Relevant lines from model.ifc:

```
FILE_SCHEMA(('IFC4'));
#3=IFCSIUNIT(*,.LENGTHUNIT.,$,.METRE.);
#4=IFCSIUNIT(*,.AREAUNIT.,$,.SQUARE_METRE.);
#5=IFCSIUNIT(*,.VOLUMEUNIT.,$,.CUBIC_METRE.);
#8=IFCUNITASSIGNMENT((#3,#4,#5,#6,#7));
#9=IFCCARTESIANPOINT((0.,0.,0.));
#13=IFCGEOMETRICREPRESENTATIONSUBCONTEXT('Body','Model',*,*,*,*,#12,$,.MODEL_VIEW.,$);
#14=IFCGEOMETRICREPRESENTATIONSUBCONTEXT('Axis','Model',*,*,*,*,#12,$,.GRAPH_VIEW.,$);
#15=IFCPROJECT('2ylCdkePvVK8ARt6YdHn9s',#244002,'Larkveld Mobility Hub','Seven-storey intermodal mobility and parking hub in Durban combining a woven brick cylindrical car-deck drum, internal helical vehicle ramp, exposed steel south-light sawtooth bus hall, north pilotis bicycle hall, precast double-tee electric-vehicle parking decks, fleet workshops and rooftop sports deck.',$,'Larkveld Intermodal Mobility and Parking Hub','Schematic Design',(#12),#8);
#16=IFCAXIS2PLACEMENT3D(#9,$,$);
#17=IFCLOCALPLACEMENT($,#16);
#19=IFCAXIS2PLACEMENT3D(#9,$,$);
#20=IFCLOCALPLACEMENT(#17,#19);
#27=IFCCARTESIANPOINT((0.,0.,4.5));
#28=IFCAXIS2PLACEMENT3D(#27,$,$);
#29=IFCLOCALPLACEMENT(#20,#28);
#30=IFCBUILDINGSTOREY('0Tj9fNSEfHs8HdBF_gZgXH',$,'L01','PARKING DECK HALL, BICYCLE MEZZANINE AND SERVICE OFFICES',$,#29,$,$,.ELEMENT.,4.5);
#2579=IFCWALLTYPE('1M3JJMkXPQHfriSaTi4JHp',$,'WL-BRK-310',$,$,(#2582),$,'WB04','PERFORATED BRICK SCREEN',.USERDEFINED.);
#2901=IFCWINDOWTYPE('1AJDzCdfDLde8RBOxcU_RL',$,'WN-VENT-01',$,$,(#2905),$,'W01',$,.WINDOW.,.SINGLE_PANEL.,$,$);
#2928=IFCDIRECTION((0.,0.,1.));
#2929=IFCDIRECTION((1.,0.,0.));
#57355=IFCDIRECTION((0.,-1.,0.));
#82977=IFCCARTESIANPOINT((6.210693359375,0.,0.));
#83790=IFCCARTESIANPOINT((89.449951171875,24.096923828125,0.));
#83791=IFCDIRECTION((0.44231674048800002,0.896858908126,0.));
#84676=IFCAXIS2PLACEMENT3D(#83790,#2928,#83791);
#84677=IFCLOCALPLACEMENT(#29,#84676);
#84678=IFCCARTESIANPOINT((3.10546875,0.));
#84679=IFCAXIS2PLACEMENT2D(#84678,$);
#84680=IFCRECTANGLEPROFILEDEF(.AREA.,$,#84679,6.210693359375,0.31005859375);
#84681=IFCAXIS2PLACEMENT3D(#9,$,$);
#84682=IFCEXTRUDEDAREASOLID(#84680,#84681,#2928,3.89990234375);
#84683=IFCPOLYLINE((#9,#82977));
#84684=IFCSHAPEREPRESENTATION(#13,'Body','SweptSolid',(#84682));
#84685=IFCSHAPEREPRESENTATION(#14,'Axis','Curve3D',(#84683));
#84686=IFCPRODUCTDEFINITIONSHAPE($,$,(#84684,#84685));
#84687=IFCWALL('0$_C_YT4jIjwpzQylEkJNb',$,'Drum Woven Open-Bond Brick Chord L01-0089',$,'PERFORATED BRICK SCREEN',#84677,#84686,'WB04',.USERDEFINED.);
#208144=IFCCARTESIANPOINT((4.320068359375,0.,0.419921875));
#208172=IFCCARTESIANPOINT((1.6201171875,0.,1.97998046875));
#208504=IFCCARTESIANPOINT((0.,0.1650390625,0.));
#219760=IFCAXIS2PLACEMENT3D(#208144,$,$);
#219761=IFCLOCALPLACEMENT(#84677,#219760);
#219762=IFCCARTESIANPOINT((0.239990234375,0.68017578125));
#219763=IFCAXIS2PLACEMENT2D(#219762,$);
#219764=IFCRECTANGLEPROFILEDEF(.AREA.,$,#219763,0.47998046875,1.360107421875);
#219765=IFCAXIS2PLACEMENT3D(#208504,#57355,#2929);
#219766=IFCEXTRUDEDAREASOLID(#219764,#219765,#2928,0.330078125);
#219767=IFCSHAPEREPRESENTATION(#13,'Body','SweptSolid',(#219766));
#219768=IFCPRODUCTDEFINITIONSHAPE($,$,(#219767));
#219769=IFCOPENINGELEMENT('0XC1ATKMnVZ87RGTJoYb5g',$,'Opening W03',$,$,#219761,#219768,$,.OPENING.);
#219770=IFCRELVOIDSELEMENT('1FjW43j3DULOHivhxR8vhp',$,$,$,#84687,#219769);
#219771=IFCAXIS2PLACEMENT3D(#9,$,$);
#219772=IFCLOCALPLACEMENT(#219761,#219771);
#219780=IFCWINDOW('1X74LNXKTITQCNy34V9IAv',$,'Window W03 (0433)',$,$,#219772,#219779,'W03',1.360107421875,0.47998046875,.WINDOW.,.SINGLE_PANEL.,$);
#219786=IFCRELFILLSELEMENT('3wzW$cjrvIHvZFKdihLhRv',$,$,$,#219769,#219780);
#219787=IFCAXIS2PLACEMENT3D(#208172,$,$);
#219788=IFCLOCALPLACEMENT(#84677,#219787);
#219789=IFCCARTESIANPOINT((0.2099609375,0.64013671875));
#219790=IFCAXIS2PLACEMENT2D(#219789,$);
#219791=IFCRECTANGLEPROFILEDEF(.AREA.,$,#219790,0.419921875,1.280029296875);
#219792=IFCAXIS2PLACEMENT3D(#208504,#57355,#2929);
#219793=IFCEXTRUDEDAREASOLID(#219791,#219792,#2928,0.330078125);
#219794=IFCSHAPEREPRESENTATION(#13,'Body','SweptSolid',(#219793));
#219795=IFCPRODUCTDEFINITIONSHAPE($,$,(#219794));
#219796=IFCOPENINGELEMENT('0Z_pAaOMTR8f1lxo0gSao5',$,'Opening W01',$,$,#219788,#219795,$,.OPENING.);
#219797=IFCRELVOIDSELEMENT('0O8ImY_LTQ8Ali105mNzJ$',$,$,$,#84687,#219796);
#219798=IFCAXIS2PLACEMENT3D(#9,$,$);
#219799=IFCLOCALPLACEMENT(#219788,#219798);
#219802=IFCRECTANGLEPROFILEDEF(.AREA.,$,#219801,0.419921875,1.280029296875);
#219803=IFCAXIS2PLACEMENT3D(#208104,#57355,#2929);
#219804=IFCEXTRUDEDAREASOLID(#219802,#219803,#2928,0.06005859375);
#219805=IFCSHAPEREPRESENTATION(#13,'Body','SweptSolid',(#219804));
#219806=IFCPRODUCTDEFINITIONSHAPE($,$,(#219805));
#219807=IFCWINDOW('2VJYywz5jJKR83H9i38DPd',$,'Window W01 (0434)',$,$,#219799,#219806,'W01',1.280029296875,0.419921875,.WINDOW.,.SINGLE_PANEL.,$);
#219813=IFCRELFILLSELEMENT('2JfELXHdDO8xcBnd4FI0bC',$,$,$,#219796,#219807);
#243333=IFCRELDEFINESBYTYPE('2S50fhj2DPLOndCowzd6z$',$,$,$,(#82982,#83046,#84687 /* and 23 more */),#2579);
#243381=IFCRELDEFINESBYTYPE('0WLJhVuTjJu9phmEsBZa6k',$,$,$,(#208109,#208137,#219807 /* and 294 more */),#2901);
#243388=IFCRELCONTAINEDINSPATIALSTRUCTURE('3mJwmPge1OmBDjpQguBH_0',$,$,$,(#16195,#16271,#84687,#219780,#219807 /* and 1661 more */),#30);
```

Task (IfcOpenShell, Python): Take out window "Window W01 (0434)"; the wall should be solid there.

```python
import ifcopenshell
import ifcopenshell.api.feature
import ifcopenshell.api.root
import ifcopenshell.geom
import ifcopenshell.util.shape

model = ifcopenshell.open("model.ifc")
settings = ifcopenshell.geom.settings()


def volume(element):
    """Net volume in cubic metres, openings subtracted."""
    shape = ifcopenshell.geom.create_shape(settings, element)
    return ifcopenshell.util.shape.get_volume(shape.geometry)


window = model.by_id(219807)
opening = window.FillsVoids[0].RelatingOpeningElement
wall = opening.VoidsElements[0].RelatingBuildingElement
before = volume(wall)

ifcopenshell.api.root.remove_product(model, product=window)
ifcopenshell.api.feature.remove_feature(model, feature=opening)

after = volume(wall)

print(f"wall volume {before:.3f} -> {after:.3f} m3")

model.write("model_updated.ifc")
```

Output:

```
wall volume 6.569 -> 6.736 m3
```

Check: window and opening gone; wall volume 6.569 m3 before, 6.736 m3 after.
